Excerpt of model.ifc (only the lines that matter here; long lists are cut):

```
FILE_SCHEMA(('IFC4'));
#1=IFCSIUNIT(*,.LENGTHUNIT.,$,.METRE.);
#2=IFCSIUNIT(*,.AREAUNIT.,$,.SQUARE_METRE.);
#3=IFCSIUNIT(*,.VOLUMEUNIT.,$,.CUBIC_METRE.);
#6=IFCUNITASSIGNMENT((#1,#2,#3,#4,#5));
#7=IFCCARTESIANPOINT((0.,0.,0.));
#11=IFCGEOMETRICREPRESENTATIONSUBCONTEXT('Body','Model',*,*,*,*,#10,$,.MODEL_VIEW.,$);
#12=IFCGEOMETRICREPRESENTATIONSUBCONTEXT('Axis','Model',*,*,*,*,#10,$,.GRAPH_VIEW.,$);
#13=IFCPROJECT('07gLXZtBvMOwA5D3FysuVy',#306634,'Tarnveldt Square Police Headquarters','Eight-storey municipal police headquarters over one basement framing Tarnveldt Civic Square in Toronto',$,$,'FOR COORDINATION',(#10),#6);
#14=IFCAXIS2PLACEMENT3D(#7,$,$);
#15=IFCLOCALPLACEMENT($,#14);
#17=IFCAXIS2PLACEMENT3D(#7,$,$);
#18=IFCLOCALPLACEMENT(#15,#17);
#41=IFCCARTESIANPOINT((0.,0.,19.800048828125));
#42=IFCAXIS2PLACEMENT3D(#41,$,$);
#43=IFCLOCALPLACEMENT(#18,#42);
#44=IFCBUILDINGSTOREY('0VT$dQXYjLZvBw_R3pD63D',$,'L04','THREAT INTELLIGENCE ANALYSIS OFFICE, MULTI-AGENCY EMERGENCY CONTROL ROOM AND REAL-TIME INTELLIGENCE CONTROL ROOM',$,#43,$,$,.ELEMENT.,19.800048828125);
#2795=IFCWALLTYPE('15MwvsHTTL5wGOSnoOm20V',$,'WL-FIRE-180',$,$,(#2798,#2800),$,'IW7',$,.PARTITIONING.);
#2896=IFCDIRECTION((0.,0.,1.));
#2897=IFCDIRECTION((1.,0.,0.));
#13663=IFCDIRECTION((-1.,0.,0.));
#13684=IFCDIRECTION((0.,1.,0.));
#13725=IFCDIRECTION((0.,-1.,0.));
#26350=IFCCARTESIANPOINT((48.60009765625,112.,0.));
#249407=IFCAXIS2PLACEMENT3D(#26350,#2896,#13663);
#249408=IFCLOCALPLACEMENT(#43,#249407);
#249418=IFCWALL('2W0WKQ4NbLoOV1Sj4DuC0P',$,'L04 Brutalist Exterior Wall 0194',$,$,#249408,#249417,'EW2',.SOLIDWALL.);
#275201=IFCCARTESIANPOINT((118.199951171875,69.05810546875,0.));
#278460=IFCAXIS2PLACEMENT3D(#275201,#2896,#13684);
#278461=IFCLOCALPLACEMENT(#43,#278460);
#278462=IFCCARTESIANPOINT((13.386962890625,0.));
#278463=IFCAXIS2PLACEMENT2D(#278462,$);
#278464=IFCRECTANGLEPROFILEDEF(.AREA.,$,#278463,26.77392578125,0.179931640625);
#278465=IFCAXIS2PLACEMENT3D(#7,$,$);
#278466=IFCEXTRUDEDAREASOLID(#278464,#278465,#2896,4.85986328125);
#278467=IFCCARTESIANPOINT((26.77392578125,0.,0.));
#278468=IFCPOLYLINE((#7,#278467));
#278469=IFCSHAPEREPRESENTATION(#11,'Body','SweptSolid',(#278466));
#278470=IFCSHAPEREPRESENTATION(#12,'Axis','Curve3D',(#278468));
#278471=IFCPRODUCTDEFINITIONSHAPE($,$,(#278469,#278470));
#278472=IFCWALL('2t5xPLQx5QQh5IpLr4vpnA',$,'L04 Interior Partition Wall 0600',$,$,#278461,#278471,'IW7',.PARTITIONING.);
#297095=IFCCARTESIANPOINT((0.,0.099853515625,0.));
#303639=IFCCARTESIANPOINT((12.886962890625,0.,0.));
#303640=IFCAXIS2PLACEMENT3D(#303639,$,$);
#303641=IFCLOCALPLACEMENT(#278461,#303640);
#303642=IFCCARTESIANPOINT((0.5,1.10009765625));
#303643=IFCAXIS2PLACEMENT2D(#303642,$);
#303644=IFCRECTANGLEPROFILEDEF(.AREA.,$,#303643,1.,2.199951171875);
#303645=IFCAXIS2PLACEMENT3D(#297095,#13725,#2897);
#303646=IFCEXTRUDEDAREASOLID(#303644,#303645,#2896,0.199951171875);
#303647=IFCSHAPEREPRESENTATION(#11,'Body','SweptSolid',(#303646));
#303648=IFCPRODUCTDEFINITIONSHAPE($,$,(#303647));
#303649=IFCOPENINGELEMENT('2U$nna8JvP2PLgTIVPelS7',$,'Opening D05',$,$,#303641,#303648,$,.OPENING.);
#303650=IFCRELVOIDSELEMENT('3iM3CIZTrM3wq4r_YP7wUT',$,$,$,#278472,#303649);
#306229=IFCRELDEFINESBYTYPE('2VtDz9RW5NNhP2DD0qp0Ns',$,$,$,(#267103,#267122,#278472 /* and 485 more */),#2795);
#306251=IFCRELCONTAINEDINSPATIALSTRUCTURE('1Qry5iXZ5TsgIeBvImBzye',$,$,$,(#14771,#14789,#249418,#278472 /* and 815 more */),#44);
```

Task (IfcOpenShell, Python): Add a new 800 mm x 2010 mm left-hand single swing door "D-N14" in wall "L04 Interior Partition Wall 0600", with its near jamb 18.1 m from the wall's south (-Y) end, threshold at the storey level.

```python
import numpy as np
import ifcopenshell
import ifcopenshell.api.feature
import ifcopenshell.api.geometry
import ifcopenshell.api.root
import ifcopenshell.api.spatial
import ifcopenshell.geom
import ifcopenshell.util.element
import ifcopenshell.util.placement
import ifcopenshell.util.representation
import ifcopenshell.util.shape
import ifcopenshell.util.unit

model = ifcopenshell.open("model.ifc")
unit_scale = ifcopenshell.util.unit.calculate_unit_scale(model)
settings = ifcopenshell.geom.settings()


def volume(element):
    """Net volume in cubic metres, openings subtracted."""
    shape = ifcopenshell.geom.create_shape(settings, element)
    return ifcopenshell.util.shape.get_volume(shape.geometry)


wall = model.by_guid("2t5xPLQx5QQh5IpLr4vpnA")
storey = ifcopenshell.util.element.get_container(wall, ifc_class="IfcBuildingStorey")
context = ifcopenshell.util.representation.get_context(model, "Model", "Body", "MODEL_VIEW")
before = volume(wall)

width, height, from_end, sill = 0.8, 2.01, 18.1, 0.0  # metres

# The wall runs along its own X axis, and the end named is its -X end.
wall_shape = ifcopenshell.geom.create_shape(settings, wall)
x, y, z = ifcopenshell.util.shape.get_vertices(wall_shape.geometry).T
start = x.min() + from_end
face, thickness = float(y.min()), float(y.max() - y.min())
wall_matrix = ifcopenshell.util.placement.get_local_placement(wall.ObjectPlacement)
level = ifcopenshell.util.placement.get_local_placement(storey.ObjectPlacement)[2, 3]


def in_wall(x, y):
    """Placement at x, y metres in the wall's axes, at sill height."""
    matrix = wall_matrix.copy()
    matrix[:, 3] = wall_matrix @ np.array([x / unit_scale, y / unit_scale, 0.0, 1.0])
    matrix[2, 3] = level + sill / unit_scale
    return matrix


# Opening: a box that overshoots both wall faces by 50 mm.
opening = ifcopenshell.api.root.create_entity(model, ifc_class="IfcOpeningElement", predefined_type="OPENING")
box = ifcopenshell.api.geometry.add_wall_representation(
    model, context=context, length=width, height=height, thickness=thickness + 0.1
)
ifcopenshell.api.geometry.assign_representation(model, product=opening, representation=box)
ifcopenshell.api.geometry.edit_object_placement(model, product=opening, matrix=in_wall(start, face - 0.05), is_si=False)
ifcopenshell.api.feature.add_feature(model, feature=opening, element=wall)

door = ifcopenshell.api.root.create_entity(model, ifc_class="IfcDoor", name="D-N14", predefined_type="DOOR")
door.OverallWidth, door.OverallHeight = width / unit_scale, height / unit_scale
door.OperationType = "SINGLE_SWING_LEFT"
body = ifcopenshell.api.geometry.add_door_representation(
    model,
    context=context,
    overall_width=door.OverallWidth,
    overall_height=door.OverallHeight,
    operation_type="SINGLE_SWING_LEFT",
    lining_properties={"LiningDepth": thickness / unit_scale, "ThresholdDepth": thickness / unit_scale},
)
ifcopenshell.api.geometry.assign_representation(model, product=door, representation=body)
ifcopenshell.api.spatial.assign_container(model, products=[door], relating_structure=storey)
ifcopenshell.api.feature.add_filling(model, opening=opening, element=door)

# The lining spans the wall, so the door starts at the wall face.
ifcopenshell.api.geometry.edit_object_placement(model, product=door, matrix=in_wall(start, face), is_si=False)

after = volume(wall)

print(f"wall volume {before:.3f} -> {after:.3f} m3")

model.write("model_edited.ifc")
```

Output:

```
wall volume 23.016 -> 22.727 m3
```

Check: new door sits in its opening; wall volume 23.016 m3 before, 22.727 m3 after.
